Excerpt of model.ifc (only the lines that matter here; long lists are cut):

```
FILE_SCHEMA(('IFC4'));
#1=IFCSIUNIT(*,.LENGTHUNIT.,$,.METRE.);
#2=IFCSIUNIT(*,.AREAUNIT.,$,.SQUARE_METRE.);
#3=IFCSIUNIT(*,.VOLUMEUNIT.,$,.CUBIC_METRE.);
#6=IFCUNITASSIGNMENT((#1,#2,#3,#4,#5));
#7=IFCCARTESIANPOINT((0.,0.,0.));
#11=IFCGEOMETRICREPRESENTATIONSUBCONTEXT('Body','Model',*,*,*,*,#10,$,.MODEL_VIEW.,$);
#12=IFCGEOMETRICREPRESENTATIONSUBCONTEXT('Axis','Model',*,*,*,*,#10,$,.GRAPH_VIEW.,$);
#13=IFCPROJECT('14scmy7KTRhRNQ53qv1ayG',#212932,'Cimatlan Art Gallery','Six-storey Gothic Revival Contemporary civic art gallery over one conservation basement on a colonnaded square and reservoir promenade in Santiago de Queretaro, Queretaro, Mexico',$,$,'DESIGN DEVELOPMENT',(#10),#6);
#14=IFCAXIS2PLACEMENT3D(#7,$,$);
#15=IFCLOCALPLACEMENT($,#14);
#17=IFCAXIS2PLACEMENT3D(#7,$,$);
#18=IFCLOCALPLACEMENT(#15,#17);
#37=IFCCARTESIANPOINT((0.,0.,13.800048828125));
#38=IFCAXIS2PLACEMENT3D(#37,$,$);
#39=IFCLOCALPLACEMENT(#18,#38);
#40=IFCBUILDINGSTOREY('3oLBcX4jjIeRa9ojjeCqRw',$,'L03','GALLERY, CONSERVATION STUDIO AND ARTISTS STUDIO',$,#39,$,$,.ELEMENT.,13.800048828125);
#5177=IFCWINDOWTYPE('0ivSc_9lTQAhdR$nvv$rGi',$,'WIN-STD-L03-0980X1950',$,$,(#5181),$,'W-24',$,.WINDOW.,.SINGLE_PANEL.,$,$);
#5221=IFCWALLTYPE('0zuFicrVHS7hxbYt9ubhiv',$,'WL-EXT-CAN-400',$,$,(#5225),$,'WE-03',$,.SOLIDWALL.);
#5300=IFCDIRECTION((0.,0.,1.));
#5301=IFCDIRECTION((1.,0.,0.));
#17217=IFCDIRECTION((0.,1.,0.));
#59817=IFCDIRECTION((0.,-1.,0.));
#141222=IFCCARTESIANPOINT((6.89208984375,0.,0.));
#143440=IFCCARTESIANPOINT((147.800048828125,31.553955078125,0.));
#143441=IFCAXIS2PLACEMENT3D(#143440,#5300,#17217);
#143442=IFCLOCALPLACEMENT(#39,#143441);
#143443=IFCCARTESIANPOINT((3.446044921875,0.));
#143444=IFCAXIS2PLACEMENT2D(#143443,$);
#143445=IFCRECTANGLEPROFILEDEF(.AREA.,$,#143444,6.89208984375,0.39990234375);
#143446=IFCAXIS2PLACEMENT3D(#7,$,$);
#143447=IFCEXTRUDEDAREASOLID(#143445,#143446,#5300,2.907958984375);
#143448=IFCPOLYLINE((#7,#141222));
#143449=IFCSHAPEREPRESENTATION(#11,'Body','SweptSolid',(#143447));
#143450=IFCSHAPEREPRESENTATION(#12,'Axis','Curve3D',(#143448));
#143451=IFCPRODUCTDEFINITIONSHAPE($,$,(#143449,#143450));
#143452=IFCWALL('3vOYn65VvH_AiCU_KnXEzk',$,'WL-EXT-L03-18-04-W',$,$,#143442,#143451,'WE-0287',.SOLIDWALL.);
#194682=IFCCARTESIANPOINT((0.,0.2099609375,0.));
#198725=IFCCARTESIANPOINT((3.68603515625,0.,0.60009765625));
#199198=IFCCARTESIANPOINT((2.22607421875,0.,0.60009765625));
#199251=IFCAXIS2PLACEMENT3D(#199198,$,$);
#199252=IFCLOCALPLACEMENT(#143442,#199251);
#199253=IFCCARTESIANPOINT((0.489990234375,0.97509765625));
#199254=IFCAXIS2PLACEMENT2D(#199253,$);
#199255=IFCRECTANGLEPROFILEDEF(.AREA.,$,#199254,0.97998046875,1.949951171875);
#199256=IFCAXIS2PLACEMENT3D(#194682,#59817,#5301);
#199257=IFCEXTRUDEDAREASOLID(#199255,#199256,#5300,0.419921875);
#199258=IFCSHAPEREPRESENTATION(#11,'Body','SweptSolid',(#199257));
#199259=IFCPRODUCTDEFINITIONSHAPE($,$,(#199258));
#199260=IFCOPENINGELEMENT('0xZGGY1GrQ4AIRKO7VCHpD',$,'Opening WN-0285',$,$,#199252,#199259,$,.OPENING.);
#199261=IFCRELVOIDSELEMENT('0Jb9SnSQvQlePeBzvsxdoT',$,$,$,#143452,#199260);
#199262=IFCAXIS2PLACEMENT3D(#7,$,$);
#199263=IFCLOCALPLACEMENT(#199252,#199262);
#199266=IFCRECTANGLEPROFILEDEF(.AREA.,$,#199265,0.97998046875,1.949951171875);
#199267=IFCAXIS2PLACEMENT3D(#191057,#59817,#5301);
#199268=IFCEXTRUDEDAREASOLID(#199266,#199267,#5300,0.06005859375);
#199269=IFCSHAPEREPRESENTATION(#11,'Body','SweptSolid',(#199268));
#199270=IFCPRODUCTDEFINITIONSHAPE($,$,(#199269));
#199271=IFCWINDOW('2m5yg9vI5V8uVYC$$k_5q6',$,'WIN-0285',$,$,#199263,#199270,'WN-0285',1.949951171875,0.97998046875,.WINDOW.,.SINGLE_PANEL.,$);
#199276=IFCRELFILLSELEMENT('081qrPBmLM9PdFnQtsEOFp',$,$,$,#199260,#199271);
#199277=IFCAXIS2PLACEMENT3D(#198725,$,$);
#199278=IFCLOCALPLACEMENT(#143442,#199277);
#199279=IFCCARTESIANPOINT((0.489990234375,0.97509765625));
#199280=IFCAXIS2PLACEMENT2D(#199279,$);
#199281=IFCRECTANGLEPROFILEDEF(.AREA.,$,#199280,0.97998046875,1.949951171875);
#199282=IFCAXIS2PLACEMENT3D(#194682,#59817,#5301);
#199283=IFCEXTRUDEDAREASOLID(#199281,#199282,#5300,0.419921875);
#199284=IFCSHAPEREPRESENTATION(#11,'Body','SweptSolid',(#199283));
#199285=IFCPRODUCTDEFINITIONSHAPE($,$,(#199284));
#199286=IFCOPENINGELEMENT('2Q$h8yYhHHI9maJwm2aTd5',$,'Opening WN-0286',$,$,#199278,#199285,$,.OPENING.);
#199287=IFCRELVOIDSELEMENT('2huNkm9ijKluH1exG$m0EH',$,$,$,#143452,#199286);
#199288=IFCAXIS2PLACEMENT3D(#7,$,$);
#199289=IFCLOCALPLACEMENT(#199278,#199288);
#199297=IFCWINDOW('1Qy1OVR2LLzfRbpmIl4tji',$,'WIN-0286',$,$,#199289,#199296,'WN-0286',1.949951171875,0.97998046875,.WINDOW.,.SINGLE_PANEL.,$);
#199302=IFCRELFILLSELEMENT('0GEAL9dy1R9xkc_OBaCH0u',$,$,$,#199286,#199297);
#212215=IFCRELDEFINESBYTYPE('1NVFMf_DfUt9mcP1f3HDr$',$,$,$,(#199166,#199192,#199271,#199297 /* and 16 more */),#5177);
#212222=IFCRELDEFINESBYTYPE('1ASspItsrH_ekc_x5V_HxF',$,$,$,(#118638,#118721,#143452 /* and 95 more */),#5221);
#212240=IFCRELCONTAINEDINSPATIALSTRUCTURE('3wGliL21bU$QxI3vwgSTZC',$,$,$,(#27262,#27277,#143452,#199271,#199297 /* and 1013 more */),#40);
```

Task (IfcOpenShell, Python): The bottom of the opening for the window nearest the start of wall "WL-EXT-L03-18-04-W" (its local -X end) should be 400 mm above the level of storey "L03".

```python
import numpy as np
import ifcopenshell
import ifcopenshell.api.geometry
import ifcopenshell.geom
import ifcopenshell.util.element
import ifcopenshell.util.placement
import ifcopenshell.util.shape
import ifcopenshell.util.unit

model = ifcopenshell.open("model.ifc")
unit_scale = ifcopenshell.util.unit.calculate_unit_scale(model)

window = model.by_guid("2m5yg9vI5V8uVYC$$k_5q6")
opening = window.FillsVoids[0].RelatingOpeningElement
storey = ifcopenshell.util.element.get_container(window, ifc_class="IfcBuildingStorey")
level = ifcopenshell.util.placement.get_local_placement(storey.ObjectPlacement)[2, 3]

# The opening's origin need not be at the sill, so measure its lowest point.
shape = ifcopenshell.geom.create_shape(ifcopenshell.geom.settings(), opening)
bottom = ifcopenshell.util.shape.get_shape_bottom_elevation(shape, shape.geometry) / unit_scale
dz = level + 0.4 - bottom

shift = np.array([0.0, 0.0, dz])
# The window is placed relative to its opening, so it follows when the opening moves.
matrix = ifcopenshell.util.placement.get_local_placement(opening.ObjectPlacement)
matrix[:3, 3] += shift
ifcopenshell.api.geometry.edit_object_placement(
    model, product=opening, matrix=matrix, is_si=False, should_transform_children=True
)

print(f"moved by {dz * unit_scale:+.3f} m")

model.write("model-out.ifc")
```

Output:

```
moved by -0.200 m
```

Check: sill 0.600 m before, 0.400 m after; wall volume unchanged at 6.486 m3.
